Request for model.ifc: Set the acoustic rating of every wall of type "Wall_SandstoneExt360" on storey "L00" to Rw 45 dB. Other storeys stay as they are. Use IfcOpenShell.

First a look at what the model holds.

```python
import ifcopenshell
import ifcopenshell.util.element

model = ifcopenshell.open("model.ifc")
print(model.schema)
storey = next(s for s in model.by_type("IfcBuildingStorey") if s.Name == "L00")
walls = [e for e in ifcopenshell.util.element.get_decomposition(storey) if e.is_a("IfcWall")]
seen = {}
for e in walls:
    element_type = ifcopenshell.util.element.get_type(e)
    key = (element_type.Name if element_type != e and element_type else None, ifcopenshell.util.element.get_pset(e, "Pset_WallCommon", "AcousticRating"))
    seen[key] = seen.get(key, 0) + 1
for (name, value), count in sorted(seen.items(), key=str):
    print(count, "x", name, "|", value)
```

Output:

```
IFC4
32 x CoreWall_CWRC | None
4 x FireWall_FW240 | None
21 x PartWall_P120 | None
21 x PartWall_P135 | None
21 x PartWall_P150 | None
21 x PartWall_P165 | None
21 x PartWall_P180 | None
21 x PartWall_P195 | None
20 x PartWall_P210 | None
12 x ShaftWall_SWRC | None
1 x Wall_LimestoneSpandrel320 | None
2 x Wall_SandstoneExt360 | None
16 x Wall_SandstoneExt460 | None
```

```python
import ifcopenshell
import ifcopenshell.api.pset
import ifcopenshell.util.element

model = ifcopenshell.open("model.ifc")

storey = next(s for s in model.by_type("IfcBuildingStorey") if s.Name == "L00")
walls = [e for e in ifcopenshell.util.element.get_decomposition(storey) if e.is_a("IfcWall")]

count = 0
for e in walls:
    element_type = ifcopenshell.util.element.get_type(e)
    if element_type in (None, e) or element_type.Name != "Wall_SandstoneExt360":
        continue
    # add_pset returns the element's existing set when there is one.
    pset = ifcopenshell.api.pset.add_pset(model, product=e, name="Pset_WallCommon")
    ifcopenshell.api.pset.edit_pset(model, pset=pset, properties={"AcousticRating": "Rw 45 dB"})
    count += 1

print(count, "walls updated")

model.write("model-out.ifc")
```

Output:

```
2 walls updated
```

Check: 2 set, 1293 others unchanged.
